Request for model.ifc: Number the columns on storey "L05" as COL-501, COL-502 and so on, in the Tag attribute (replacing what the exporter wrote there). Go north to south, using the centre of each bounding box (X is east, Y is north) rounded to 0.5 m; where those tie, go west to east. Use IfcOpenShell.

First a look at what the model holds.

```python
import ifcopenshell
import ifcopenshell.util.element
import ifcopenshell.util.placement

model = ifcopenshell.open("model.ifc")
print(model.schema)
storey = next(s for s in model.by_type("IfcBuildingStorey") if s.Name == "L05")
columns = [e for e in ifcopenshell.util.element.get_decomposition(storey) if e.is_a("IfcColumn")]
for e in sorted(columns, key=lambda e: e.id()):
    origin = ifcopenshell.util.placement.get_local_placement(e.ObjectPlacement)[:3, 3]
    print(e.id(), e.Tag, e.Name, origin.round(2) + 0.0, sep=" | ")
```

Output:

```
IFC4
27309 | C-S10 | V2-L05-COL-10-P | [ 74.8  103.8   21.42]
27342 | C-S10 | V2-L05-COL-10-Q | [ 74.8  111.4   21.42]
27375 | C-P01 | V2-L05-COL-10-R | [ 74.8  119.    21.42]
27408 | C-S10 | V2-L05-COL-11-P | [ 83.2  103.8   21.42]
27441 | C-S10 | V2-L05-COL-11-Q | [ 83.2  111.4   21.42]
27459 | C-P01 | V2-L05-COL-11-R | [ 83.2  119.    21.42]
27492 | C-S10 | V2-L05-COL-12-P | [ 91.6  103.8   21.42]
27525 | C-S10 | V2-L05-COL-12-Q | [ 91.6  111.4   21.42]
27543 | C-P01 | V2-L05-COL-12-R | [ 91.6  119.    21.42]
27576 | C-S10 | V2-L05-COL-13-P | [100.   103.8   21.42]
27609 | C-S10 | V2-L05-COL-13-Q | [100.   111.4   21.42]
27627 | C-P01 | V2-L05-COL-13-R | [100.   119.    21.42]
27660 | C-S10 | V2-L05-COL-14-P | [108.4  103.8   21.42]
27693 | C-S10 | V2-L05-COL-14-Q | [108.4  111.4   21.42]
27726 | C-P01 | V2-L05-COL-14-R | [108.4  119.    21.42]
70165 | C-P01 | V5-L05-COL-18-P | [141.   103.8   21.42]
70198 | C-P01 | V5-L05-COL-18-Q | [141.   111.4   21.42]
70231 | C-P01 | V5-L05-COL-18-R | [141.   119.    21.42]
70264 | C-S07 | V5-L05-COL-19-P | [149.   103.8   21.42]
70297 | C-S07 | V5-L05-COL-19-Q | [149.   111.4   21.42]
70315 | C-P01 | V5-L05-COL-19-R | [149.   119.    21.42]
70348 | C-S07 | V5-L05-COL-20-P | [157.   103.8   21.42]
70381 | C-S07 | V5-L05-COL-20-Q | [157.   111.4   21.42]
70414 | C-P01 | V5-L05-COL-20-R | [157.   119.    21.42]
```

```python
import ifcopenshell
import ifcopenshell.geom
import ifcopenshell.util.element
import ifcopenshell.util.shape

model = ifcopenshell.open("model.ifc")
settings = ifcopenshell.geom.settings()
settings.set("use-world-coords", True)


def centre(element):
    shape = ifcopenshell.geom.create_shape(settings, element)
    return ifcopenshell.util.shape.get_bbox_centroid(shape.geometry)


storey = next(s for s in model.by_type("IfcBuildingStorey") if s.Name == "L05")
columns = [e for e in ifcopenshell.util.element.get_decomposition(storey) if e.is_a("IfcColumn")]

# Insertion points can sit at a corner or the storey origin, so sort by the geometry (in metres).
centres = {e: centre(e) for e in columns}
columns.sort(key=lambda e: (-round(centres[e][1] / 0.5), centres[e][0]))

for i, e in enumerate(columns, start=1):
    number = f"COL-5{i:02d}"
    e.Tag = number
    print(e.id(), number)

model.write("model_updated.ifc")
```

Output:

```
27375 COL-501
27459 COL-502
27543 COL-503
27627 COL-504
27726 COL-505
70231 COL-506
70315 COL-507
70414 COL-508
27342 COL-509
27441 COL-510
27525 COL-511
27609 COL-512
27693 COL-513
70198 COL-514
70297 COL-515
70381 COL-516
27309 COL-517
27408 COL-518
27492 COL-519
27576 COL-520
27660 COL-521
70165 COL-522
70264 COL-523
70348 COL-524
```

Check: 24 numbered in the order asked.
